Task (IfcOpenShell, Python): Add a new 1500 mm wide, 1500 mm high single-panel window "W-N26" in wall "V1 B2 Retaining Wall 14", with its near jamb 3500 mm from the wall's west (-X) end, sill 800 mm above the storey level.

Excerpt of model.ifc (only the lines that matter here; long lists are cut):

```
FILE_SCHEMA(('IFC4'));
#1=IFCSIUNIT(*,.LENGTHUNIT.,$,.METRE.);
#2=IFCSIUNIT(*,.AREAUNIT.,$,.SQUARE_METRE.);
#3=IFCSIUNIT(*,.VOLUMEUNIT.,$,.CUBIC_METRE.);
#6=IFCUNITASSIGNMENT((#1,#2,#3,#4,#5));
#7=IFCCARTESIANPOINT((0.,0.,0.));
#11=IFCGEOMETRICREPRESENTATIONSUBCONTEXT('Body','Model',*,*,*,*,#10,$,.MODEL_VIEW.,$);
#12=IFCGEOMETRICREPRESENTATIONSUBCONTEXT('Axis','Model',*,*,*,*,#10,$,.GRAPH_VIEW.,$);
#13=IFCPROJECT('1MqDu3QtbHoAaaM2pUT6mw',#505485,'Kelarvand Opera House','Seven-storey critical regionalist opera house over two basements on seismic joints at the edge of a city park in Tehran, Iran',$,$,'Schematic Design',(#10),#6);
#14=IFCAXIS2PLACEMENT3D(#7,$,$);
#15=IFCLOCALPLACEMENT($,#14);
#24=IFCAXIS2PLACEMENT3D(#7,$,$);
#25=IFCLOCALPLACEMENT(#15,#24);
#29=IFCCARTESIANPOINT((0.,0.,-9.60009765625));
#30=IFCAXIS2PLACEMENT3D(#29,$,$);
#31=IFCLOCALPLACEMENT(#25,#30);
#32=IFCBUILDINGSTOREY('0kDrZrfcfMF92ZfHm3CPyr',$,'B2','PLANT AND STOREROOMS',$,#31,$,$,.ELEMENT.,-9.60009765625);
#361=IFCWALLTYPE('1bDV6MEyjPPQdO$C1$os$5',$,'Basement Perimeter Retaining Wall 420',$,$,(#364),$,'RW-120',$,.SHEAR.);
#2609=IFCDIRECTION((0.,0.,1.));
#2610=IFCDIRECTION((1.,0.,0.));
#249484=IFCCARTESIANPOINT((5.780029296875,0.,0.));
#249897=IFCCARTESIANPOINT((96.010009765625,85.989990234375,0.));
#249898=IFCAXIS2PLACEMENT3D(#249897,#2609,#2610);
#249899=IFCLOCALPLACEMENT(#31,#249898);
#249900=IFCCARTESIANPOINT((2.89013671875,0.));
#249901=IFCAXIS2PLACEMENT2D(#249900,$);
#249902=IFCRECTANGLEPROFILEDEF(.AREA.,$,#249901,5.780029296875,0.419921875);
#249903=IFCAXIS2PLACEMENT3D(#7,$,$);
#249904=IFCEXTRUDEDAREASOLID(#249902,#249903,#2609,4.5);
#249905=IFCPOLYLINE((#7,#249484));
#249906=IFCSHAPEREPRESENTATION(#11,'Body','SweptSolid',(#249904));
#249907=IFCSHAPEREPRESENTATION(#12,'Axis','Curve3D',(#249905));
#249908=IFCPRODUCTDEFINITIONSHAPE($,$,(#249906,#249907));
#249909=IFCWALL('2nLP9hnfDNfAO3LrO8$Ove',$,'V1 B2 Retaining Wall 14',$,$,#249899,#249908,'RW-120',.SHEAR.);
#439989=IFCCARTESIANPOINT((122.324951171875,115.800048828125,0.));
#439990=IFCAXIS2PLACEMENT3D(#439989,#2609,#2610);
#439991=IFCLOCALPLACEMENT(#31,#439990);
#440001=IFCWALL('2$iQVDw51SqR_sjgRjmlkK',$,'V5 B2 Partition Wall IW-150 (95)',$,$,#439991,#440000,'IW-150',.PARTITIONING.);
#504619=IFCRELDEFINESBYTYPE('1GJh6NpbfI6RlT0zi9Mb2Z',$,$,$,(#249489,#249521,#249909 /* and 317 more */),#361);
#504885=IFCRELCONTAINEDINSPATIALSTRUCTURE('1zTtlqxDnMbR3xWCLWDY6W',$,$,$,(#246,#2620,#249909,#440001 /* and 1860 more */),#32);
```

```python
import numpy as np
import ifcopenshell
import ifcopenshell.api.feature
import ifcopenshell.api.geometry
import ifcopenshell.api.root
import ifcopenshell.api.spatial
import ifcopenshell.geom
import ifcopenshell.util.element
import ifcopenshell.util.placement
import ifcopenshell.util.representation
import ifcopenshell.util.shape
import ifcopenshell.util.unit

model = ifcopenshell.open("model.ifc")
unit_scale = ifcopenshell.util.unit.calculate_unit_scale(model)
settings = ifcopenshell.geom.settings()


def volume(element):
    """Net volume in cubic metres, openings subtracted."""
    shape = ifcopenshell.geom.create_shape(settings, element)
    return ifcopenshell.util.shape.get_volume(shape.geometry)


wall = model.by_guid("2nLP9hnfDNfAO3LrO8$Ove")
storey = ifcopenshell.util.element.get_container(wall, ifc_class="IfcBuildingStorey")
context = ifcopenshell.util.representation.get_context(model, "Model", "Body", "MODEL_VIEW")
before = volume(wall)

width, height, from_end, sill = 1.5, 1.5, 3.5, 0.8  # metres

# The wall runs along its own X axis, and the end named is its -X end.
wall_shape = ifcopenshell.geom.create_shape(settings, wall)
x, y, z = ifcopenshell.util.shape.get_vertices(wall_shape.geometry).T
start = x.min() + from_end
face, thickness = float(y.min()), float(y.max() - y.min())
wall_matrix = ifcopenshell.util.placement.get_local_placement(wall.ObjectPlacement)
level = ifcopenshell.util.placement.get_local_placement(storey.ObjectPlacement)[2, 3]


def in_wall(x, y):
    """Placement at x, y metres in the wall's axes, at sill height."""
    matrix = wall_matrix.copy()
    matrix[:, 3] = wall_matrix @ np.array([x / unit_scale, y / unit_scale, 0.0, 1.0])
    matrix[2, 3] = level + sill / unit_scale
    return matrix


# Opening: a box that overshoots both wall faces by 50 mm.
opening = ifcopenshell.api.root.create_entity(model, ifc_class="IfcOpeningElement", predefined_type="OPENING")
box = ifcopenshell.api.geometry.add_wall_representation(
    model, context=context, length=width, height=height, thickness=thickness + 0.1
)
ifcopenshell.api.geometry.assign_representation(model, product=opening, representation=box)
ifcopenshell.api.geometry.edit_object_placement(model, product=opening, matrix=in_wall(start, face - 0.05), is_si=False)
ifcopenshell.api.feature.add_feature(model, feature=opening, element=wall)

window = ifcopenshell.api.root.create_entity(model, ifc_class="IfcWindow", name="W-N26", predefined_type="WINDOW")
window.OverallWidth, window.OverallHeight = width / unit_scale, height / unit_scale
window.PartitioningType = "SINGLE_PANEL"
body = ifcopenshell.api.geometry.add_window_representation(
    model,
    context=context,
    overall_width=window.OverallWidth,
    overall_height=window.OverallHeight,
    partition_type="SINGLE_PANEL",
)
ifcopenshell.api.geometry.assign_representation(model, product=window, representation=body)
ifcopenshell.api.spatial.assign_container(model, products=[window], relating_structure=storey)
ifcopenshell.api.feature.add_filling(model, opening=opening, element=window)

# Centre the window in the wall's thickness.
ifcopenshell.api.geometry.edit_object_placement(model, product=window, matrix=in_wall(start, face), is_si=False)
window_shape = ifcopenshell.geom.create_shape(settings, window)
depth = ifcopenshell.util.shape.get_vertices(window_shape.geometry)[:, 1]
offset = face + thickness / 2 - (depth.min() + depth.max()) / 2
ifcopenshell.api.geometry.edit_object_placement(model, product=window, matrix=in_wall(start, offset), is_si=False)

after = volume(wall)

print(f"wall volume {before:.3f} -> {after:.3f} m3")

model.write("model_rev.ifc")
```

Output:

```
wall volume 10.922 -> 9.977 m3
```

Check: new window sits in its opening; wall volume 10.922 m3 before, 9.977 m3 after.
